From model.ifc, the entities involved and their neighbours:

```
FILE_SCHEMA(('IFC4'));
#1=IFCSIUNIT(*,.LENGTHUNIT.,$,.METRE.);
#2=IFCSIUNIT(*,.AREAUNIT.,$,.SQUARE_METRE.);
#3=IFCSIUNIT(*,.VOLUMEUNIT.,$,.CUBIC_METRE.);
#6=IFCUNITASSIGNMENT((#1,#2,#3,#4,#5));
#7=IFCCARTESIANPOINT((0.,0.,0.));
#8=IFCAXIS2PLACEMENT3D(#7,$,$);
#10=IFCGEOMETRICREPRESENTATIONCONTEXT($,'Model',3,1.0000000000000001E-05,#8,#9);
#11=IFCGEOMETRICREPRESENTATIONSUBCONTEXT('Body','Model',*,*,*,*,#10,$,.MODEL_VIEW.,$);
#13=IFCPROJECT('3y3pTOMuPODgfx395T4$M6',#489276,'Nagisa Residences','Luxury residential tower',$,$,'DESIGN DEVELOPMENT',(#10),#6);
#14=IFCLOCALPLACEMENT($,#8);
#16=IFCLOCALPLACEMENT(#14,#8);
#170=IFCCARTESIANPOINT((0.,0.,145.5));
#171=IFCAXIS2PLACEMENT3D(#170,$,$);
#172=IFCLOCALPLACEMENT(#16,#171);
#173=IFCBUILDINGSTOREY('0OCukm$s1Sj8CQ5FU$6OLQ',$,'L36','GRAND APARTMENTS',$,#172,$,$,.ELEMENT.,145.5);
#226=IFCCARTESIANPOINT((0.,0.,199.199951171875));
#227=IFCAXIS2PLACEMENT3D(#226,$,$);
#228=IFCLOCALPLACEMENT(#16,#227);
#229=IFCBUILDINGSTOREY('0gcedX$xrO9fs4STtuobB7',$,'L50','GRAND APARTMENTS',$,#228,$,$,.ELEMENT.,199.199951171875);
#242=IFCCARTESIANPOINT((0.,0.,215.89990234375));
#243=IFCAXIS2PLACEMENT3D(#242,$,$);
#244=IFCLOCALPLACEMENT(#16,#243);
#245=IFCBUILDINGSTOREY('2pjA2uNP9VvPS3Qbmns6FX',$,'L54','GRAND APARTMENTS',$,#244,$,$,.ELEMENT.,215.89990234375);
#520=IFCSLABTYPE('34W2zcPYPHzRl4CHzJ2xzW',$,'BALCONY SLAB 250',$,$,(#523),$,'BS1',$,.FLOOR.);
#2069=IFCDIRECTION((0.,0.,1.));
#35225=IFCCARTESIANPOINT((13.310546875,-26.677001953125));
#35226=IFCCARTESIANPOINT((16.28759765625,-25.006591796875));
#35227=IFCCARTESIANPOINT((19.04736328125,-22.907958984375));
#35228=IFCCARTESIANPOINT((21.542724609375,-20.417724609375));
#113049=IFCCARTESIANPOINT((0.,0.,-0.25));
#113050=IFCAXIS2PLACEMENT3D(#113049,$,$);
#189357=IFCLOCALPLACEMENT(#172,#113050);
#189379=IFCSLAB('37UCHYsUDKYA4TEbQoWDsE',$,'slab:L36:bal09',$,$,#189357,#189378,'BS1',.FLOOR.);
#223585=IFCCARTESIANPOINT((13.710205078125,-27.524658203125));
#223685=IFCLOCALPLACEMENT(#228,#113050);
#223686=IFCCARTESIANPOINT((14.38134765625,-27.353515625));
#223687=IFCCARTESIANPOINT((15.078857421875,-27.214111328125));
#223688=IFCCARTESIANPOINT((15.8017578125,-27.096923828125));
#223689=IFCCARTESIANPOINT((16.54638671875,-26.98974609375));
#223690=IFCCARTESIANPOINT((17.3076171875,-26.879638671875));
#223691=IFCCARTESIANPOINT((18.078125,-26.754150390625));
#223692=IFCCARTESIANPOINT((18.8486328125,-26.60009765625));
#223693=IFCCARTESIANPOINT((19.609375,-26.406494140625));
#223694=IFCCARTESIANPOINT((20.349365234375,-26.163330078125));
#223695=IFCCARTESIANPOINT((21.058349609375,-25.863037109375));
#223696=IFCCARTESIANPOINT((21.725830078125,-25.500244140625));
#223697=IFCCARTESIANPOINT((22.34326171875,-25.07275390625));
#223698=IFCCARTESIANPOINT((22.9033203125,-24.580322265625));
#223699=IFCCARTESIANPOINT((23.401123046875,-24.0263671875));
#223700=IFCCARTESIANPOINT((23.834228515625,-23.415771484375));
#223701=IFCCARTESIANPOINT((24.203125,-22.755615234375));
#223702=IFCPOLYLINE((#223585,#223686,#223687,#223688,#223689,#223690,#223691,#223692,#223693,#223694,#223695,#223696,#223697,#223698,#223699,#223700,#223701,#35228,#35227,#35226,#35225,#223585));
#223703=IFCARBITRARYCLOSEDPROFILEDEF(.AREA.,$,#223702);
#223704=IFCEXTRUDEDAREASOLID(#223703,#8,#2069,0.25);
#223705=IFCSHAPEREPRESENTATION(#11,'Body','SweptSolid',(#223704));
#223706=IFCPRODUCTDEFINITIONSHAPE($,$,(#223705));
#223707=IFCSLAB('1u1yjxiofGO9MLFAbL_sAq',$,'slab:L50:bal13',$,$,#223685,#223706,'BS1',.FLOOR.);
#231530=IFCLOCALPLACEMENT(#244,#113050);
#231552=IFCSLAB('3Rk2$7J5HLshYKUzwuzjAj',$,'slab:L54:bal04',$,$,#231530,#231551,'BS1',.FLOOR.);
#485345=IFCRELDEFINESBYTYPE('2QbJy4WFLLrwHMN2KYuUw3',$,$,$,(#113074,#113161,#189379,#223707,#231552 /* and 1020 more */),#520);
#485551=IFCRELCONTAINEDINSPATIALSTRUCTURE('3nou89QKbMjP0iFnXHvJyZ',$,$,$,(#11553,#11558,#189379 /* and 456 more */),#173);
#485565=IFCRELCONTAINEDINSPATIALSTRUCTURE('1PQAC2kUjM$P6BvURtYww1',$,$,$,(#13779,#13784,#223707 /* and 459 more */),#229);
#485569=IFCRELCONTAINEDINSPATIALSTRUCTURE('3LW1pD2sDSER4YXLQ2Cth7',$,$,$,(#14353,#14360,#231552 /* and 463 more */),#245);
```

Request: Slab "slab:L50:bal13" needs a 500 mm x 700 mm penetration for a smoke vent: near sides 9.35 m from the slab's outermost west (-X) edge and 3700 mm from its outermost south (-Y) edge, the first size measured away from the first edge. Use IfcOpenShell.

```python
import numpy as np
import ifcopenshell
import ifcopenshell.api.feature
import ifcopenshell.api.geometry
import ifcopenshell.api.root
import ifcopenshell.geom
import ifcopenshell.util.placement
import ifcopenshell.util.representation
import ifcopenshell.util.shape
import ifcopenshell.util.unit

model = ifcopenshell.open("model.ifc")
unit_scale = ifcopenshell.util.unit.calculate_unit_scale(model)
settings = ifcopenshell.geom.settings()


def volume(element):
    """Net volume in cubic metres, openings subtracted."""
    shape = ifcopenshell.geom.create_shape(settings, element)
    return ifcopenshell.util.shape.get_volume(shape.geometry)


slab = model.by_id(223707)
before = volume(slab)

# Extent in the slab's own axes, in metres. The edges named are its -X and -Y sides.
slab_shape = ifcopenshell.geom.create_shape(settings, slab)
vertices = ifcopenshell.util.shape.get_vertices(slab_shape.geometry)
x_min, y_min, bottom = vertices.min(axis=0)
top = vertices[:, 2].max()

opening = ifcopenshell.api.root.create_entity(model, ifc_class="IfcOpeningElement", name="Smoke vent opening", predefined_type="OPENING")
context = ifcopenshell.util.representation.get_context(model, "Model", "Body", "MODEL_VIEW")
width, depth = 0.5, 0.7
outline = [(0.0, 0.0), (width, 0.0), (width, depth), (0.0, depth), (0.0, 0.0)]
# Overshoot both faces by 50 mm so the cut is clean.
shape = ifcopenshell.api.geometry.add_slab_representation(
    model, context=context, depth=top - bottom + 0.1, polyline=outline
)
ifcopenshell.api.geometry.assign_representation(model, product=opening, representation=shape)

matrix = ifcopenshell.util.placement.get_local_placement(slab.ObjectPlacement)
matrix[:, 3] = matrix @ np.append(np.array([x_min + 9.35, y_min + 3.7, bottom - 0.05]) / unit_scale, 1.0)
ifcopenshell.api.geometry.edit_object_placement(model, product=opening, matrix=matrix, is_si=False)
ifcopenshell.api.feature.add_feature(model, feature=opening, element=slab)

after = volume(slab)

print(f"slab volume {before:.3f} -> {after:.3f} m3")

model.write("model_rev.ifc")
```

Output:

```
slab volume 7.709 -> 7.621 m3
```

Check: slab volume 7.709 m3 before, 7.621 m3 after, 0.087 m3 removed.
